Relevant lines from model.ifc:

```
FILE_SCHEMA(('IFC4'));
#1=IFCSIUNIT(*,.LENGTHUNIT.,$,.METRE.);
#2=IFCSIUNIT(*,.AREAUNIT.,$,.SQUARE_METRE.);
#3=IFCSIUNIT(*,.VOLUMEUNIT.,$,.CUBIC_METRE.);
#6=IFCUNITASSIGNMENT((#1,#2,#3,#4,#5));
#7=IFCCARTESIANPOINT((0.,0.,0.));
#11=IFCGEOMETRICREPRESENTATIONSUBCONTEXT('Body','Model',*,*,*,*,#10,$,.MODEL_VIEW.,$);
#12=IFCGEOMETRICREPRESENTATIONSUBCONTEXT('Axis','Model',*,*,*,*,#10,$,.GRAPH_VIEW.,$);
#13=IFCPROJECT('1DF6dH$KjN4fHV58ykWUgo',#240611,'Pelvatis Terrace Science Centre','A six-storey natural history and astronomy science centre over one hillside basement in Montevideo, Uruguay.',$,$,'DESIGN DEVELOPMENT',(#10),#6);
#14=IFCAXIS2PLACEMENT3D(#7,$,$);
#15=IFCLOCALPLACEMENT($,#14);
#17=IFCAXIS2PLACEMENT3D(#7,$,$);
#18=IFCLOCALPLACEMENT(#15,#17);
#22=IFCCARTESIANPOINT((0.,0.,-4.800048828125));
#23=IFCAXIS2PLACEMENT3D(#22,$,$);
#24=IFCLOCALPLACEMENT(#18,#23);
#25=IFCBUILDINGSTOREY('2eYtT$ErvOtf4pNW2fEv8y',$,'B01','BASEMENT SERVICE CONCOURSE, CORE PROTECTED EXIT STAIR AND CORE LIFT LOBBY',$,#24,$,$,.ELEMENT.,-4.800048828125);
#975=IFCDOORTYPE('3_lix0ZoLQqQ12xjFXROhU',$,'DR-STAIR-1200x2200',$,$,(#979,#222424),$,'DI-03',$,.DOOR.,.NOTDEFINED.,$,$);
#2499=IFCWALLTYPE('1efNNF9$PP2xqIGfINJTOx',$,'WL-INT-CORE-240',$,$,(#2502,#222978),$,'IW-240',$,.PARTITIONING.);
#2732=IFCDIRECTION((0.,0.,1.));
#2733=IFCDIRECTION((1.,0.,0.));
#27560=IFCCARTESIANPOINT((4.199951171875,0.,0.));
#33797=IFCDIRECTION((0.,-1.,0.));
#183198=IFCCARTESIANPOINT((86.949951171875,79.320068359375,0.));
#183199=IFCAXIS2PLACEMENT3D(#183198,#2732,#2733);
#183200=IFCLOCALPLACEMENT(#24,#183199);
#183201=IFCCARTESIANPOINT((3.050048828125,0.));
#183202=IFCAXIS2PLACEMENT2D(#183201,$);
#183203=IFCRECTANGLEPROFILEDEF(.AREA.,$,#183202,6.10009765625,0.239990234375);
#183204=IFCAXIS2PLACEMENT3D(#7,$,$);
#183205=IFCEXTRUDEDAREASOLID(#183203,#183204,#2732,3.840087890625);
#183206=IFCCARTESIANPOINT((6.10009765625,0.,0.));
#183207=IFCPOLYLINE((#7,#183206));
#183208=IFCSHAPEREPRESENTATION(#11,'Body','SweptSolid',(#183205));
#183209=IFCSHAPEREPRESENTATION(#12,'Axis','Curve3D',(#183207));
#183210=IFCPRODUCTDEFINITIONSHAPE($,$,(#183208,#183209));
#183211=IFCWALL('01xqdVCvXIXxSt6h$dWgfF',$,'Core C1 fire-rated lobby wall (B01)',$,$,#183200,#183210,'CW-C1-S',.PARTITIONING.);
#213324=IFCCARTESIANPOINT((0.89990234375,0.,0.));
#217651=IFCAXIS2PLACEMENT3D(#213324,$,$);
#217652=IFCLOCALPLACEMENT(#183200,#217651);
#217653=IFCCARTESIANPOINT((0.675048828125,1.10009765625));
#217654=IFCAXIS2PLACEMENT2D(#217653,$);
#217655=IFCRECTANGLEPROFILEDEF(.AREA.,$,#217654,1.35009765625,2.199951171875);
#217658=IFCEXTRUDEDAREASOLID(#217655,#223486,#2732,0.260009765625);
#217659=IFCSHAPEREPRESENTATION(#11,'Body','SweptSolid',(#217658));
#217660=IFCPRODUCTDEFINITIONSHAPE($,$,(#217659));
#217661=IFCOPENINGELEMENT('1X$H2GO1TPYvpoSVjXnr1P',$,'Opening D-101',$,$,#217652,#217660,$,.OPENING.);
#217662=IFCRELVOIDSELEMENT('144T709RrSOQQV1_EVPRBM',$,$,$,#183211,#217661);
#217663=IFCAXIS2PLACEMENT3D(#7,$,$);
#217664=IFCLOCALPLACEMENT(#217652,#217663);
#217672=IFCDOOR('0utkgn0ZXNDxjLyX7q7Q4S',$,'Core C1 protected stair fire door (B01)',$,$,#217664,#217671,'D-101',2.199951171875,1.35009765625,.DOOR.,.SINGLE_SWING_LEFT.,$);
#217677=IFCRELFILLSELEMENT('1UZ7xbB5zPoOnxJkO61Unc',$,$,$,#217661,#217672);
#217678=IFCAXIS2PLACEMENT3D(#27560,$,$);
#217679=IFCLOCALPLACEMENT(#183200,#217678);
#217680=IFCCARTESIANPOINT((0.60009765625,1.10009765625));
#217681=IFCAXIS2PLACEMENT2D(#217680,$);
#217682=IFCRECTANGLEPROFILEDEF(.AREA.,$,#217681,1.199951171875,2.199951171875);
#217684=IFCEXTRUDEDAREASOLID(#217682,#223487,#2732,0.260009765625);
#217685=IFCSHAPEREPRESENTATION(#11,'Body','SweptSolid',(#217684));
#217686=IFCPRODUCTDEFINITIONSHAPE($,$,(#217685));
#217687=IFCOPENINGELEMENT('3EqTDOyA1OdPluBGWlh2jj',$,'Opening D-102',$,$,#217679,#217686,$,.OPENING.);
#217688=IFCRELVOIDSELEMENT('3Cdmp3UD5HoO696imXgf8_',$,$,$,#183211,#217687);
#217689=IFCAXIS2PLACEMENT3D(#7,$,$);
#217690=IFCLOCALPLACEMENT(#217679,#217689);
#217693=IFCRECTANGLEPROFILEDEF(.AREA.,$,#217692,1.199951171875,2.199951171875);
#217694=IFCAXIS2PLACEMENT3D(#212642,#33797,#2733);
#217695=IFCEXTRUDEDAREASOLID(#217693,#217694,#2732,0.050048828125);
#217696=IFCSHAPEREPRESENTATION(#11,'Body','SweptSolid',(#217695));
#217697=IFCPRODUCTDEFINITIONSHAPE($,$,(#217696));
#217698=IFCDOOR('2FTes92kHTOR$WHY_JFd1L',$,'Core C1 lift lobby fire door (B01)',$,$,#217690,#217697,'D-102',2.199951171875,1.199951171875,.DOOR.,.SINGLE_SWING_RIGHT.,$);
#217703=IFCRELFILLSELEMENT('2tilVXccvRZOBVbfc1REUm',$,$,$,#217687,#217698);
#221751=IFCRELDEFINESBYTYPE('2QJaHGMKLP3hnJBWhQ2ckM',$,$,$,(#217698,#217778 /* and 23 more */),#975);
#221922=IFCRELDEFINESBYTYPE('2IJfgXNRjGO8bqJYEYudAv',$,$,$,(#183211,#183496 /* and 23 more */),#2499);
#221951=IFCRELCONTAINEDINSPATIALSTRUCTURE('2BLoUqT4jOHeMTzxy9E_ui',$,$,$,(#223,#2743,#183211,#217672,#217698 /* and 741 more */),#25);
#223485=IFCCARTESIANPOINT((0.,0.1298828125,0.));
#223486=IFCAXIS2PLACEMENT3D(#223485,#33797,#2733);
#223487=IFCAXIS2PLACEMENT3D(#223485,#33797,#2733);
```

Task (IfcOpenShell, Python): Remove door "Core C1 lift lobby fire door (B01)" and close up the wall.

```python
import ifcopenshell
import ifcopenshell.api.feature
import ifcopenshell.api.root
import ifcopenshell.geom
import ifcopenshell.util.shape

model = ifcopenshell.open("model.ifc")
settings = ifcopenshell.geom.settings()


def volume(element):
    """Net volume in cubic metres, openings subtracted."""
    shape = ifcopenshell.geom.create_shape(settings, element)
    return ifcopenshell.util.shape.get_volume(shape.geometry)


door = model.by_guid("2FTes92kHTOR$WHY_JFd1L")
opening = door.FillsVoids[0].RelatingOpeningElement
wall = opening.VoidsElements[0].RelatingBuildingElement
before = volume(wall)

ifcopenshell.api.root.remove_product(model, product=door)
ifcopenshell.api.feature.remove_feature(model, feature=opening)

after = volume(wall)

print(f"wall volume {before:.3f} -> {after:.3f} m3")

model.write("model_updated.ifc")
```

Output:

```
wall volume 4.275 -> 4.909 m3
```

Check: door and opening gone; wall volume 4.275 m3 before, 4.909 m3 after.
